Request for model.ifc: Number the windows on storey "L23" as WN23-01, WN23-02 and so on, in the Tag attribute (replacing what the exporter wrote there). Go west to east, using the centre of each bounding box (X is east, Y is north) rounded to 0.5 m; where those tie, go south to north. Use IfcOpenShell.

First a look at what the model holds.

```python
import ifcopenshell
import ifcopenshell.util.element
import ifcopenshell.util.placement

model = ifcopenshell.open("model.ifc")
print(model.schema)
storey = next(s for s in model.by_type("IfcBuildingStorey") if s.Name == "L23")
windows = [e for e in ifcopenshell.util.element.get_decomposition(storey) if e.is_a("IfcWindow")]
for e in sorted(windows, key=lambda e: e.id()):
    origin = ifcopenshell.util.placement.get_local_placement(e.ObjectPlacement)[:3, 3]
    print(e.id(), e.Tag, e.Name, origin.round(2) + 0.0, sep=" | ")
```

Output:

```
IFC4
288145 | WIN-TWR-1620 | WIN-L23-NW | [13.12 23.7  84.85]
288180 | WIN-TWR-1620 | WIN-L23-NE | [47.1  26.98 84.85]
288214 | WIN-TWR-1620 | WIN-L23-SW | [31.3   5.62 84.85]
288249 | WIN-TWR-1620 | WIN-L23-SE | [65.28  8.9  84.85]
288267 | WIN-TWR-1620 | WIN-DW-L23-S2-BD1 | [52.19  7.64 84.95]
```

```python
import ifcopenshell
import ifcopenshell.geom
import ifcopenshell.util.element
import ifcopenshell.util.shape

model = ifcopenshell.open("model.ifc")
settings = ifcopenshell.geom.settings()
settings.set("use-world-coords", True)


def centre(element):
    shape = ifcopenshell.geom.create_shape(settings, element)
    return ifcopenshell.util.shape.get_bbox_centroid(shape.geometry)


storey = next(s for s in model.by_type("IfcBuildingStorey") if s.Name == "L23")
windows = [e for e in ifcopenshell.util.element.get_decomposition(storey) if e.is_a("IfcWindow")]

# Insertion points can sit at a corner or the storey origin, so sort by the geometry (in metres).
centres = {e: centre(e) for e in windows}
windows.sort(key=lambda e: (round(centres[e][0] / 0.5), centres[e][1]))

for i, e in enumerate(windows, start=1):
    number = f"WN23-{i:02d}"
    e.Tag = number
    print(e.id(), number)

model.write("model-out.ifc")
```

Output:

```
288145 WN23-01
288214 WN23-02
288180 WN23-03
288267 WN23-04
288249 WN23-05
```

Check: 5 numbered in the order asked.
